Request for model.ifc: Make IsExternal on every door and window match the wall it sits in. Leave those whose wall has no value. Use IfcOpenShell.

First a look at what the model holds.

```python
import ifcopenshell
import ifcopenshell.util.element

model = ifcopenshell.open("model.ifc")
print(model.schema)
seen = {}
for e in model.by_type("IfcDoor") + model.by_type("IfcWindow"):
    if not e.FillsVoids:
        continue
    host = e.FillsVoids[0].RelatingOpeningElement.VoidsElements[0].RelatingBuildingElement
    own = ifcopenshell.util.element.get_pset(e, f"Pset_{e.is_a()[3:].removesuffix('StandardCase')}Common", "IsExternal")
    wall = ifcopenshell.util.element.get_pset(host, "Pset_WallCommon", "IsExternal")
    seen[e.is_a(), own, wall] = seen.get((e.is_a(), own, wall), 0) + 1
for (cls, own, wall), count in sorted(seen.items(), key=str):
    print(count, cls, "IsExternal:", own, "| host wall:", wall)
```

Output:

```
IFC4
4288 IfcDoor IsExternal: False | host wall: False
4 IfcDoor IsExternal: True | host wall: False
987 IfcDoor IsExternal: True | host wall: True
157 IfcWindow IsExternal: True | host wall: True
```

```python
import ifcopenshell
import ifcopenshell.api.pset
import ifcopenshell.util.element

model = ifcopenshell.open("model.ifc")

count = 0
for ifc_class, pset_name in (("IfcDoor", "Pset_DoorCommon"), ("IfcWindow", "Pset_WindowCommon")):
    for e in model.by_type(ifc_class):
        if not e.FillsVoids:
            continue
        host = e.FillsVoids[0].RelatingOpeningElement.VoidsElements[0].RelatingBuildingElement
        external = ifcopenshell.util.element.get_pset(host, "Pset_WallCommon", "IsExternal")
        if external is None or ifcopenshell.util.element.get_pset(e, pset_name, "IsExternal") == external:
            continue
        pset = ifcopenshell.api.pset.add_pset(model, product=e, name=pset_name)
        ifcopenshell.api.pset.edit_pset(model, pset=pset, properties={"IsExternal": external})
        count += 1

print(count, "updated")

model.write("model_rev.ifc")
```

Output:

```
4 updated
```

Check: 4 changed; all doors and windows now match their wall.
